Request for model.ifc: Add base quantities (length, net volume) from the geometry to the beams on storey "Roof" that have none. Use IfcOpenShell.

First a look at what the model holds.

```python
import ifcopenshell
import ifcopenshell.util.element
import ifcopenshell.util.unit

model = ifcopenshell.open("model.ifc")
print(model.schema)
for unit_type in ("LENGTHUNIT", "AREAUNIT", "VOLUMEUNIT"):
    print(unit_type, ifcopenshell.util.unit.calculate_unit_scale(model, unit_type))
storey = next(s for s in model.by_type("IfcBuildingStorey") if s.Name == "Roof")
beams = [e for e in ifcopenshell.util.element.get_decomposition(storey) if e.is_a("IfcBeam")]
for e in sorted(beams, key=lambda e: e.id()):
    print(e.id(), e.is_a(), e.Name, list(ifcopenshell.util.element.get_psets(e, qtos_only=True)), sep=" | ")
```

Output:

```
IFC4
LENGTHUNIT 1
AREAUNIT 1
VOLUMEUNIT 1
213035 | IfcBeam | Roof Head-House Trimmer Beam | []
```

```python
import ifcopenshell
import ifcopenshell.api.pset
import ifcopenshell.geom
import ifcopenshell.util.element
import ifcopenshell.util.shape
import ifcopenshell.util.unit

model = ifcopenshell.open("model.ifc")
unit_scale = ifcopenshell.util.unit.calculate_unit_scale(model)
volume_scale = ifcopenshell.util.unit.calculate_unit_scale(model, "VOLUMEUNIT")
settings = ifcopenshell.geom.settings()

storey = next(s for s in model.by_type("IfcBuildingStorey") if s.Name == "Roof")
beams = [e for e in ifcopenshell.util.element.get_decomposition(storey) if e.is_a("IfcBeam")]

for e in sorted(beams, key=lambda e: e.id()):
    if ifcopenshell.util.element.get_psets(e, qtos_only=True, should_inherit=False):
        continue
    # Geometry comes back in metres, in the element's own axes.
    shape = ifcopenshell.geom.create_shape(settings, e)
    values = {
        "Length": ifcopenshell.util.shape.get_max_xyz(shape.geometry) / unit_scale,
        "NetVolume": ifcopenshell.util.shape.get_volume(shape.geometry) / volume_scale,
    }
    qto = ifcopenshell.api.pset.add_qto(model, product=e, name="Qto_BeamBaseQuantities")
    ifcopenshell.api.pset.edit_qto(model, qto=qto, properties=values)
    print(e.id(), {k: round(v, 3) for k, v in values.items()})

model.write("model_updated.ifc")
```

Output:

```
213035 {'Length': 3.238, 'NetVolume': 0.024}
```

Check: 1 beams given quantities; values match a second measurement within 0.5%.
